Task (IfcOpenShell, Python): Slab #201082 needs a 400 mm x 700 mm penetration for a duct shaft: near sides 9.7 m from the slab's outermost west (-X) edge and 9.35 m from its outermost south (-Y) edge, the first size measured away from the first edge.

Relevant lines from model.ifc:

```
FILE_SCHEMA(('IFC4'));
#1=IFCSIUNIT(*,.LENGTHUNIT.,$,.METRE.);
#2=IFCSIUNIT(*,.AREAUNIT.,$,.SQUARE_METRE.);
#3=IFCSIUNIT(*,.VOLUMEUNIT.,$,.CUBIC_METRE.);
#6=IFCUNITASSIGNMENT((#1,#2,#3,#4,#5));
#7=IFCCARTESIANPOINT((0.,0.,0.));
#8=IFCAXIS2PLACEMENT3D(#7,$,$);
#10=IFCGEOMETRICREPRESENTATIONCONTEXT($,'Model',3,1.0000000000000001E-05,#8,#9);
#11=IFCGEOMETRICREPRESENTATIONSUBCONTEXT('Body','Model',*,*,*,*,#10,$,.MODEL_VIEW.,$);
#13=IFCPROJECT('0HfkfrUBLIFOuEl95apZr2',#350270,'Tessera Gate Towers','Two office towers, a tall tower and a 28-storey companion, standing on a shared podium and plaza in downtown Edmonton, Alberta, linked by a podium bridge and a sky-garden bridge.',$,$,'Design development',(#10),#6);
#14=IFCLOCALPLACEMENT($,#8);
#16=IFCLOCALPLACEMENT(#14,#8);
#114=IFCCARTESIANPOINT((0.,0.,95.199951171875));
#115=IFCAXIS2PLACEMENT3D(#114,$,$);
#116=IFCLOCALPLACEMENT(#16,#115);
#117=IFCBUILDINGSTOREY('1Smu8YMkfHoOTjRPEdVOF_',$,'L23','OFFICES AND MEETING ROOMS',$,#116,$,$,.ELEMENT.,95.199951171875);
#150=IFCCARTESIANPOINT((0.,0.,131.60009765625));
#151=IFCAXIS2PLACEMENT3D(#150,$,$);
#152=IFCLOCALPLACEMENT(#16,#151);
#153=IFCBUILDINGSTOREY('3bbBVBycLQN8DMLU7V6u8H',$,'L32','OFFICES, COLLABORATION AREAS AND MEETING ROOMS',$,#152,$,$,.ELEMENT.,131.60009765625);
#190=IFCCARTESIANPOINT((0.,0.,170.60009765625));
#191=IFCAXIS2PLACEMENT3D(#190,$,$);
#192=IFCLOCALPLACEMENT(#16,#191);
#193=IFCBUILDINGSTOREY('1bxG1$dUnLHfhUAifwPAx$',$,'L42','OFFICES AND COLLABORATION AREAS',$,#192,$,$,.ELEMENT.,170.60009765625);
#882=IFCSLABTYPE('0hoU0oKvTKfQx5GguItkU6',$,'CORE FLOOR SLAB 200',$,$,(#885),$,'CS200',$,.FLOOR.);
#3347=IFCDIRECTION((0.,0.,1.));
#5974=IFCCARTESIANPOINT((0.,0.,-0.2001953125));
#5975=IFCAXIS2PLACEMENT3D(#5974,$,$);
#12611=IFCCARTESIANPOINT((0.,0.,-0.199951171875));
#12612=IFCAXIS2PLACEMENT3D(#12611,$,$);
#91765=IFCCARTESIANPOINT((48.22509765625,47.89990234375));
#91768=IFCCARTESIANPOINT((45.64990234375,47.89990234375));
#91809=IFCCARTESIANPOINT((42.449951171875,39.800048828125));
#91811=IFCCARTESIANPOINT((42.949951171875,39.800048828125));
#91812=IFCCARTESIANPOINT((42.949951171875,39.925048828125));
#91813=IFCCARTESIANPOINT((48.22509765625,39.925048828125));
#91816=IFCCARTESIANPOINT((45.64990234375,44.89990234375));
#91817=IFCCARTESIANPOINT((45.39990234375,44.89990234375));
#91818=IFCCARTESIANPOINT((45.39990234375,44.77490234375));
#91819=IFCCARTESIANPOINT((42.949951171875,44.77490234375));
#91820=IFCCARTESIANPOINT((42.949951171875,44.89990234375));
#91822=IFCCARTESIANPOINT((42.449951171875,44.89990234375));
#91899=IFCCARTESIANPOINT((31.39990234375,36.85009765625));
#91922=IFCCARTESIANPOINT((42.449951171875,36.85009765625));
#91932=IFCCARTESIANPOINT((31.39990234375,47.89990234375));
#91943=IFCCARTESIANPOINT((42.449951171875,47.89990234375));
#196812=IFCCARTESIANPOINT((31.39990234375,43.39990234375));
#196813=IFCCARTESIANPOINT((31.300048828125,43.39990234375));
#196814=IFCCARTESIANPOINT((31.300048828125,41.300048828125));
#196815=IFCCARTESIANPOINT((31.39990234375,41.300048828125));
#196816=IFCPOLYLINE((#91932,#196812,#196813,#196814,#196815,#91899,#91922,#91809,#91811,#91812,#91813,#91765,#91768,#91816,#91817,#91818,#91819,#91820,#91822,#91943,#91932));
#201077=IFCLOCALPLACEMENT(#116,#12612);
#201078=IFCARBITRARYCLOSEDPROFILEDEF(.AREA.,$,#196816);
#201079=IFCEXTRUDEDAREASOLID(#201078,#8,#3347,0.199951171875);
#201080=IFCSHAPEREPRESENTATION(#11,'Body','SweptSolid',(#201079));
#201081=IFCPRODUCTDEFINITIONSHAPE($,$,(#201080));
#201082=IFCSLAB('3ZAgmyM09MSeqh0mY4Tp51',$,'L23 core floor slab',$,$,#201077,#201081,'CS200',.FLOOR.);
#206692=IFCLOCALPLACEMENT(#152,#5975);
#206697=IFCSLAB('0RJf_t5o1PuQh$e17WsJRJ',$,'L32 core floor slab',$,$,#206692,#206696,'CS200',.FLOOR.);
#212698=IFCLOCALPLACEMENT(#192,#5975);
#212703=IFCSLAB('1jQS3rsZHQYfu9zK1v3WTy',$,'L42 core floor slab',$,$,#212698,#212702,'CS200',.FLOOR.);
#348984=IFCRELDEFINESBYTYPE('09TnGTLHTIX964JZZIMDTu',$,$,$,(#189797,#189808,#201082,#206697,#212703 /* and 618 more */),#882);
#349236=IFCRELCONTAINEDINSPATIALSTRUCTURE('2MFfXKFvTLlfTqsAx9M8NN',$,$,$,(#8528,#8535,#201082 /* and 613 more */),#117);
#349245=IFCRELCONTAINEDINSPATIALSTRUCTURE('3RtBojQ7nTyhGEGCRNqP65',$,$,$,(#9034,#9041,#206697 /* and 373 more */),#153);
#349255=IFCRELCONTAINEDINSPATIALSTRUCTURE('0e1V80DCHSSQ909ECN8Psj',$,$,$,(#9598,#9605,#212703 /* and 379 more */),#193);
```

```python
import numpy as np
import ifcopenshell
import ifcopenshell.api.feature
import ifcopenshell.api.geometry
import ifcopenshell.api.root
import ifcopenshell.geom
import ifcopenshell.util.placement
import ifcopenshell.util.representation
import ifcopenshell.util.shape
import ifcopenshell.util.unit

model = ifcopenshell.open("model.ifc")
unit_scale = ifcopenshell.util.unit.calculate_unit_scale(model)
settings = ifcopenshell.geom.settings()


def volume(element):
    """Net volume in cubic metres, openings subtracted."""
    shape = ifcopenshell.geom.create_shape(settings, element)
    return ifcopenshell.util.shape.get_volume(shape.geometry)


slab = model.by_id(201082)
before = volume(slab)

# Extent in the slab's own axes, in metres. The edges named are its -X and -Y sides.
slab_shape = ifcopenshell.geom.create_shape(settings, slab)
vertices = ifcopenshell.util.shape.get_vertices(slab_shape.geometry)
x_min, y_min, bottom = vertices.min(axis=0)
top = vertices[:, 2].max()

opening = ifcopenshell.api.root.create_entity(model, ifc_class="IfcOpeningElement", name="Duct shaft opening", predefined_type="OPENING")
context = ifcopenshell.util.representation.get_context(model, "Model", "Body", "MODEL_VIEW")
width, depth = 0.4, 0.7
outline = [(0.0, 0.0), (width, 0.0), (width, depth), (0.0, depth), (0.0, 0.0)]
# Overshoot both faces by 50 mm so the cut is clean.
shape = ifcopenshell.api.geometry.add_slab_representation(
    model, context=context, depth=top - bottom + 0.1, polyline=outline
)
ifcopenshell.api.geometry.assign_representation(model, product=opening, representation=shape)

matrix = ifcopenshell.util.placement.get_local_placement(slab.ObjectPlacement)
matrix[:, 3] = matrix @ np.append(np.array([x_min + 9.7, y_min + 9.35, bottom - 0.05]) / unit_scale, 1.0)
ifcopenshell.api.geometry.edit_object_placement(model, product=opening, matrix=matrix, is_si=False)
ifcopenshell.api.feature.add_feature(model, feature=opening, element=slab)

after = volume(slab)

print(f"slab volume {before:.3f} -> {after:.3f} m3")

model.write("model_edited.ifc")
```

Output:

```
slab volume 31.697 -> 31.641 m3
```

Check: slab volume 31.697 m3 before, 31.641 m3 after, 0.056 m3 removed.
